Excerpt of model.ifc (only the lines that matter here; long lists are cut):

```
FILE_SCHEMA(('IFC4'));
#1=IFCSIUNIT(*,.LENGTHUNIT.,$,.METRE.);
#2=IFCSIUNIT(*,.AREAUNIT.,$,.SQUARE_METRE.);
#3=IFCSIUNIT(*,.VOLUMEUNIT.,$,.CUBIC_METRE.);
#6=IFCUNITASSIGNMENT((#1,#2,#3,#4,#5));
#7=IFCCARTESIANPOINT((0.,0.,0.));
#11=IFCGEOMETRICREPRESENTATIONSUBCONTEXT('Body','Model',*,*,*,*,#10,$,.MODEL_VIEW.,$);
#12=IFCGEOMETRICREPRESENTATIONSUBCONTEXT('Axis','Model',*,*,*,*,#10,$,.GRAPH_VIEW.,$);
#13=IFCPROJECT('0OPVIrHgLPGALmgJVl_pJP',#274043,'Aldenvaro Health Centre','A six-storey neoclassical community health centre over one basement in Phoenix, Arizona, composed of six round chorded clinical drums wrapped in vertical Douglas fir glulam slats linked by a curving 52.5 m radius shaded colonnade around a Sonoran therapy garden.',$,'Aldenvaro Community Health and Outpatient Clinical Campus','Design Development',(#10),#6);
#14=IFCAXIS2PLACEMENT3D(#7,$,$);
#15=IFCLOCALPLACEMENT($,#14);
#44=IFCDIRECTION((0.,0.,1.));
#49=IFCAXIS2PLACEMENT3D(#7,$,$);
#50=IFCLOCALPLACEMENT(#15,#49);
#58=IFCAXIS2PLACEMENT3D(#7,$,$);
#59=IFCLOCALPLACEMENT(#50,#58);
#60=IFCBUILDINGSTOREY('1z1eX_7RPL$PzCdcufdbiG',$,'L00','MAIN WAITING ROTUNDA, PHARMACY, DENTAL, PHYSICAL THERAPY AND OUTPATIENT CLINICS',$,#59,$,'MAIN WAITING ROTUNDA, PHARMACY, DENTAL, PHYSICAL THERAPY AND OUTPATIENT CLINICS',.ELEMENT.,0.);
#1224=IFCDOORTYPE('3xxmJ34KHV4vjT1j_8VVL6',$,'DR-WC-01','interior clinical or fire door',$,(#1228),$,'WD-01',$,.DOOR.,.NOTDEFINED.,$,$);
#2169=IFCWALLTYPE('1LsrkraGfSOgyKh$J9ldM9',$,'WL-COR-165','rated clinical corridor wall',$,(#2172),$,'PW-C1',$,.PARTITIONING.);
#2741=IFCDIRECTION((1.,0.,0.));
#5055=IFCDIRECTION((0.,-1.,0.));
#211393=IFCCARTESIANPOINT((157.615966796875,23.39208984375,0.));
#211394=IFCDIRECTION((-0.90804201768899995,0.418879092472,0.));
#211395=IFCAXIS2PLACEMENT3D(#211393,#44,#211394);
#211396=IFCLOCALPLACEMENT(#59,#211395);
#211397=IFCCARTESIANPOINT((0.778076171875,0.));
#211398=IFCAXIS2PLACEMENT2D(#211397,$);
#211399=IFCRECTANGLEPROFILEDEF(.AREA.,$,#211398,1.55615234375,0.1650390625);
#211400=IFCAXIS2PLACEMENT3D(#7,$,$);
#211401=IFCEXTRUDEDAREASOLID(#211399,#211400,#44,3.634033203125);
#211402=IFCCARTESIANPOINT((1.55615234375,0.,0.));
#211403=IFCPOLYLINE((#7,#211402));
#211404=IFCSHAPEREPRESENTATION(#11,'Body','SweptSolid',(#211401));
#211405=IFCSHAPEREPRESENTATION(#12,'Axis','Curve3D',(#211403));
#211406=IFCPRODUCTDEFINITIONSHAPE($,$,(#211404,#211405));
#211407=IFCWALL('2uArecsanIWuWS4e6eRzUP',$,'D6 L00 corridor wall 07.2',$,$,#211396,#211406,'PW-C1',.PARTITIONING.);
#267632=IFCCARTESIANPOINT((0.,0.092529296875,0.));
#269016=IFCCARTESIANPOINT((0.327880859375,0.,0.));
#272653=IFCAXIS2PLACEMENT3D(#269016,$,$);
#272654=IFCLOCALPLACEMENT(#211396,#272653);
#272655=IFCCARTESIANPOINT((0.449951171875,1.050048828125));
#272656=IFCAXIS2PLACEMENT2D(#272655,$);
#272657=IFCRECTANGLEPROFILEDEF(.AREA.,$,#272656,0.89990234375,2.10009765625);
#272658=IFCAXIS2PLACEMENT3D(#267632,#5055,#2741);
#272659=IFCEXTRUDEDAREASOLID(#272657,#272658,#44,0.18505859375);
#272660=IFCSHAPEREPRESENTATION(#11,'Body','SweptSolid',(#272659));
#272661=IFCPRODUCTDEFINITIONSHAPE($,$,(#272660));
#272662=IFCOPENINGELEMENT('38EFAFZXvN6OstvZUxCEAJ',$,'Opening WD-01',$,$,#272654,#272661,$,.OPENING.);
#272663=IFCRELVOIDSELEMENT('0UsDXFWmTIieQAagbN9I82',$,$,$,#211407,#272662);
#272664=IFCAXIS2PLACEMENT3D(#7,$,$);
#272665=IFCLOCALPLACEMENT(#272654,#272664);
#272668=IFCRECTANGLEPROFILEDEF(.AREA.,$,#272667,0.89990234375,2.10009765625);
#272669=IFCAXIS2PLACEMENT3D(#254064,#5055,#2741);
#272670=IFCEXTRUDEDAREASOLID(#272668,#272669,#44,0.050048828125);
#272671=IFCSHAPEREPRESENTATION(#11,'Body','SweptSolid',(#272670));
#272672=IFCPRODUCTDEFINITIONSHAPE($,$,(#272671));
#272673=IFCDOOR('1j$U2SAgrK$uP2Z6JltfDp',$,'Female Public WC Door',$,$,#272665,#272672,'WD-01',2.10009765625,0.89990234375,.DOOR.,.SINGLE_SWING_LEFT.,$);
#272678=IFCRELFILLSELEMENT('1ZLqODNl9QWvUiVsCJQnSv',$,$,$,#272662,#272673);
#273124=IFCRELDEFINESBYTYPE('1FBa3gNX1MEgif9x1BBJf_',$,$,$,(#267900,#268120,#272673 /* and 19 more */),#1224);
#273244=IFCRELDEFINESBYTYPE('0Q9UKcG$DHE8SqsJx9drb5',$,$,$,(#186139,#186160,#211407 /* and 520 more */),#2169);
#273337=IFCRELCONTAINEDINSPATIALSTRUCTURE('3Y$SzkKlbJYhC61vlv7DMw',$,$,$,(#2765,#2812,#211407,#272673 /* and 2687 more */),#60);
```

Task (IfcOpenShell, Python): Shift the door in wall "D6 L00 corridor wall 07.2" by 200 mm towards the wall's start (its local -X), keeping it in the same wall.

```python
import ifcopenshell
import ifcopenshell.api.geometry
import ifcopenshell.util.placement

model = ifcopenshell.open("model.ifc")

door = model.by_guid("1j$U2SAgrK$uP2Z6JltfDp")
opening = door.FillsVoids[0].RelatingOpeningElement
wall = opening.VoidsElements[0].RelatingBuildingElement

wall_matrix = ifcopenshell.util.placement.get_local_placement(wall.ObjectPlacement)
shift = wall_matrix[:3, 0] * -0.2
before = ifcopenshell.util.placement.get_local_placement(door.ObjectPlacement)[:3, 3].copy()

# The door is placed relative to its opening, so it follows when the opening moves.
matrix = ifcopenshell.util.placement.get_local_placement(opening.ObjectPlacement)
matrix[:3, 3] += shift
ifcopenshell.api.geometry.edit_object_placement(
    model, product=opening, matrix=matrix, is_si=False, should_transform_children=True
)

after = ifcopenshell.util.placement.get_local_placement(door.ObjectPlacement)[:3, 3]
print("door moved by", (after - before).round(3) + 0.0)

model.write("model-out.ifc")
```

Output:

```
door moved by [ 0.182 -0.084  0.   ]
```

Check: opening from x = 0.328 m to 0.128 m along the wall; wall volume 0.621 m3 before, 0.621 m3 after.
